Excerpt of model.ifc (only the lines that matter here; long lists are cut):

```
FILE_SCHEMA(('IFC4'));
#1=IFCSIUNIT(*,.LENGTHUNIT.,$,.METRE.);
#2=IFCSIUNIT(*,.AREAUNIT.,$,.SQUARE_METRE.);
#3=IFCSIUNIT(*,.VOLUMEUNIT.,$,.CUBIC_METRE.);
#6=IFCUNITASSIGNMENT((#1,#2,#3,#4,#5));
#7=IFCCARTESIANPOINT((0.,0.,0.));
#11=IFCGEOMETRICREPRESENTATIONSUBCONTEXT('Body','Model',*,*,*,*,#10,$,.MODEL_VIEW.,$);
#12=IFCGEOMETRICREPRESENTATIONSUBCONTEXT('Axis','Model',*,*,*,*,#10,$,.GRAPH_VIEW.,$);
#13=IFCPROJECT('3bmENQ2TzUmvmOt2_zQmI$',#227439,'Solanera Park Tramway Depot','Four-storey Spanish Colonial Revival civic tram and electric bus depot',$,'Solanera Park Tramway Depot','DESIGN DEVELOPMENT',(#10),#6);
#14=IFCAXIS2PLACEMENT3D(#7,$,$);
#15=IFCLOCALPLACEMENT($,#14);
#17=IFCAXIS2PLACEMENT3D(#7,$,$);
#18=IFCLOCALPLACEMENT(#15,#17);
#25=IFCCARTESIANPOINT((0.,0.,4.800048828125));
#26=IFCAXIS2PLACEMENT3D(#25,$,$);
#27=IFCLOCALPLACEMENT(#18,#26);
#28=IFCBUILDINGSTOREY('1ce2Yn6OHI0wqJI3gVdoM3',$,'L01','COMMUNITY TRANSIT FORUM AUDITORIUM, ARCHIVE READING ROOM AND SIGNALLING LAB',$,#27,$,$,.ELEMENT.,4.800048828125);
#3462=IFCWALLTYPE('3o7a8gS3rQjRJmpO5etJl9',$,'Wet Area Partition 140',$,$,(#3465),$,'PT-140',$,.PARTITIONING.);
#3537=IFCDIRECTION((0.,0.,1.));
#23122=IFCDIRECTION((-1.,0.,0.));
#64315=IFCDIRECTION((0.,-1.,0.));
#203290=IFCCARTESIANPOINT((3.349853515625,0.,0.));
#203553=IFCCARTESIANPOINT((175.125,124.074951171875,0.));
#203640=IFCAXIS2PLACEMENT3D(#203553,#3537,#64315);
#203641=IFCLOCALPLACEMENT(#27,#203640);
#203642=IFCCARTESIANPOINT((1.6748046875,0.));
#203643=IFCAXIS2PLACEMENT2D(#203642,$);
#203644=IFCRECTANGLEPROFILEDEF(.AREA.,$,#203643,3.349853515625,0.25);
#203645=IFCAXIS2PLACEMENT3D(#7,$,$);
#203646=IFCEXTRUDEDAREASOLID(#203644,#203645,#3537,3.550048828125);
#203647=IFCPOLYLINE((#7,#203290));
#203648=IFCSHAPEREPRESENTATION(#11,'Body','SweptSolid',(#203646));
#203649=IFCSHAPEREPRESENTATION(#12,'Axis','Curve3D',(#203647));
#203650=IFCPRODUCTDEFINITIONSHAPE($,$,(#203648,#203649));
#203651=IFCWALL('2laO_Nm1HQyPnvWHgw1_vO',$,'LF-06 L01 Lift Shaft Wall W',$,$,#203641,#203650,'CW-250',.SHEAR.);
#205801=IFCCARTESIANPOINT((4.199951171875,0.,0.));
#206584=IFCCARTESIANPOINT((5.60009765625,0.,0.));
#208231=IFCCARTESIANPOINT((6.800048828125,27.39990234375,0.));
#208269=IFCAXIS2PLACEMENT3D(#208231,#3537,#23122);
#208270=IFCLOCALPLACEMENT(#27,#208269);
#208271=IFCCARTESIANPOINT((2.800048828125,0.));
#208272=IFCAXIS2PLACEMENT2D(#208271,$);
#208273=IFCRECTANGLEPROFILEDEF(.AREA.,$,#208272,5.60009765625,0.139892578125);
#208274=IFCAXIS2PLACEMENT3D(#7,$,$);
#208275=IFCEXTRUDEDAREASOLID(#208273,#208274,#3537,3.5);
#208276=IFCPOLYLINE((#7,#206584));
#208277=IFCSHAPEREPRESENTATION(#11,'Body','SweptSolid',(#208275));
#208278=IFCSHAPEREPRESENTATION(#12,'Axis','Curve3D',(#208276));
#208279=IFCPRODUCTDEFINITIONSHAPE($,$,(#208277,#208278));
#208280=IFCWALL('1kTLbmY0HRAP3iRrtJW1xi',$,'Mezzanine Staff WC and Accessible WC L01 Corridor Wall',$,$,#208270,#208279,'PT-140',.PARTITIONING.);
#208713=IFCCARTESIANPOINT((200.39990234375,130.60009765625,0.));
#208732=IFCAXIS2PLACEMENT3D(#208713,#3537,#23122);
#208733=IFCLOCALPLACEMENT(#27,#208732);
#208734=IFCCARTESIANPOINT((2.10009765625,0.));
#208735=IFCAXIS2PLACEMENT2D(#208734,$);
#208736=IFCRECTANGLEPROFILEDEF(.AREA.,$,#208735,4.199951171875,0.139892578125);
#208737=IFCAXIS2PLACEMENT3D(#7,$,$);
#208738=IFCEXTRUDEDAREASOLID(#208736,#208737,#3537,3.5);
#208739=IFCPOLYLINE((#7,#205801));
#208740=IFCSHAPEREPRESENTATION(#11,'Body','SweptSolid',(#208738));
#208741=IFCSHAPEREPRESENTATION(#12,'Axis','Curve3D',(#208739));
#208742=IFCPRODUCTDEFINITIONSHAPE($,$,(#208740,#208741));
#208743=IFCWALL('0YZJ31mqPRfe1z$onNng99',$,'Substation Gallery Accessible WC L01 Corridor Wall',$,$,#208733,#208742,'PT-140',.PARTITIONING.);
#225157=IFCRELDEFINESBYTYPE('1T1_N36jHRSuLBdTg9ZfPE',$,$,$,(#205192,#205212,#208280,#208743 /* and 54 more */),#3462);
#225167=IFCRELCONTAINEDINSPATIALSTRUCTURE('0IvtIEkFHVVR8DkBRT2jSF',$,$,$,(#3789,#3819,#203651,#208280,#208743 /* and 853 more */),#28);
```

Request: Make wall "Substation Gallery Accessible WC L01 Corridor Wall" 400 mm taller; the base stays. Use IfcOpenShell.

```python
import ifcopenshell
import ifcopenshell.geom
import ifcopenshell.util.representation
import ifcopenshell.util.shape
import ifcopenshell.util.unit

model = ifcopenshell.open("model.ifc")
unit_scale = ifcopenshell.util.unit.calculate_unit_scale(model)
settings = ifcopenshell.geom.settings()


def volume(element):
    """Net volume in cubic metres, openings subtracted."""
    shape = ifcopenshell.geom.create_shape(settings, element)
    return ifcopenshell.util.shape.get_volume(shape.geometry)


wall = model.by_id(208743)
before = volume(wall)

body = ifcopenshell.util.representation.get_representation(wall, "Model", "Body")
solid = body.Items[0]
old_height = solid.Depth
solid.Depth += 0.4 / unit_scale
after = volume(wall)

print(f"height {old_height:g} -> {solid.Depth:g}, volume {before:.3f} -> {after:.3f} m3")

model.write("model-out.ifc")
```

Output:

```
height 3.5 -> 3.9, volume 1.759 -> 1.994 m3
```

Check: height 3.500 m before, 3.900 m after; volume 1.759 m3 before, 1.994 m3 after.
